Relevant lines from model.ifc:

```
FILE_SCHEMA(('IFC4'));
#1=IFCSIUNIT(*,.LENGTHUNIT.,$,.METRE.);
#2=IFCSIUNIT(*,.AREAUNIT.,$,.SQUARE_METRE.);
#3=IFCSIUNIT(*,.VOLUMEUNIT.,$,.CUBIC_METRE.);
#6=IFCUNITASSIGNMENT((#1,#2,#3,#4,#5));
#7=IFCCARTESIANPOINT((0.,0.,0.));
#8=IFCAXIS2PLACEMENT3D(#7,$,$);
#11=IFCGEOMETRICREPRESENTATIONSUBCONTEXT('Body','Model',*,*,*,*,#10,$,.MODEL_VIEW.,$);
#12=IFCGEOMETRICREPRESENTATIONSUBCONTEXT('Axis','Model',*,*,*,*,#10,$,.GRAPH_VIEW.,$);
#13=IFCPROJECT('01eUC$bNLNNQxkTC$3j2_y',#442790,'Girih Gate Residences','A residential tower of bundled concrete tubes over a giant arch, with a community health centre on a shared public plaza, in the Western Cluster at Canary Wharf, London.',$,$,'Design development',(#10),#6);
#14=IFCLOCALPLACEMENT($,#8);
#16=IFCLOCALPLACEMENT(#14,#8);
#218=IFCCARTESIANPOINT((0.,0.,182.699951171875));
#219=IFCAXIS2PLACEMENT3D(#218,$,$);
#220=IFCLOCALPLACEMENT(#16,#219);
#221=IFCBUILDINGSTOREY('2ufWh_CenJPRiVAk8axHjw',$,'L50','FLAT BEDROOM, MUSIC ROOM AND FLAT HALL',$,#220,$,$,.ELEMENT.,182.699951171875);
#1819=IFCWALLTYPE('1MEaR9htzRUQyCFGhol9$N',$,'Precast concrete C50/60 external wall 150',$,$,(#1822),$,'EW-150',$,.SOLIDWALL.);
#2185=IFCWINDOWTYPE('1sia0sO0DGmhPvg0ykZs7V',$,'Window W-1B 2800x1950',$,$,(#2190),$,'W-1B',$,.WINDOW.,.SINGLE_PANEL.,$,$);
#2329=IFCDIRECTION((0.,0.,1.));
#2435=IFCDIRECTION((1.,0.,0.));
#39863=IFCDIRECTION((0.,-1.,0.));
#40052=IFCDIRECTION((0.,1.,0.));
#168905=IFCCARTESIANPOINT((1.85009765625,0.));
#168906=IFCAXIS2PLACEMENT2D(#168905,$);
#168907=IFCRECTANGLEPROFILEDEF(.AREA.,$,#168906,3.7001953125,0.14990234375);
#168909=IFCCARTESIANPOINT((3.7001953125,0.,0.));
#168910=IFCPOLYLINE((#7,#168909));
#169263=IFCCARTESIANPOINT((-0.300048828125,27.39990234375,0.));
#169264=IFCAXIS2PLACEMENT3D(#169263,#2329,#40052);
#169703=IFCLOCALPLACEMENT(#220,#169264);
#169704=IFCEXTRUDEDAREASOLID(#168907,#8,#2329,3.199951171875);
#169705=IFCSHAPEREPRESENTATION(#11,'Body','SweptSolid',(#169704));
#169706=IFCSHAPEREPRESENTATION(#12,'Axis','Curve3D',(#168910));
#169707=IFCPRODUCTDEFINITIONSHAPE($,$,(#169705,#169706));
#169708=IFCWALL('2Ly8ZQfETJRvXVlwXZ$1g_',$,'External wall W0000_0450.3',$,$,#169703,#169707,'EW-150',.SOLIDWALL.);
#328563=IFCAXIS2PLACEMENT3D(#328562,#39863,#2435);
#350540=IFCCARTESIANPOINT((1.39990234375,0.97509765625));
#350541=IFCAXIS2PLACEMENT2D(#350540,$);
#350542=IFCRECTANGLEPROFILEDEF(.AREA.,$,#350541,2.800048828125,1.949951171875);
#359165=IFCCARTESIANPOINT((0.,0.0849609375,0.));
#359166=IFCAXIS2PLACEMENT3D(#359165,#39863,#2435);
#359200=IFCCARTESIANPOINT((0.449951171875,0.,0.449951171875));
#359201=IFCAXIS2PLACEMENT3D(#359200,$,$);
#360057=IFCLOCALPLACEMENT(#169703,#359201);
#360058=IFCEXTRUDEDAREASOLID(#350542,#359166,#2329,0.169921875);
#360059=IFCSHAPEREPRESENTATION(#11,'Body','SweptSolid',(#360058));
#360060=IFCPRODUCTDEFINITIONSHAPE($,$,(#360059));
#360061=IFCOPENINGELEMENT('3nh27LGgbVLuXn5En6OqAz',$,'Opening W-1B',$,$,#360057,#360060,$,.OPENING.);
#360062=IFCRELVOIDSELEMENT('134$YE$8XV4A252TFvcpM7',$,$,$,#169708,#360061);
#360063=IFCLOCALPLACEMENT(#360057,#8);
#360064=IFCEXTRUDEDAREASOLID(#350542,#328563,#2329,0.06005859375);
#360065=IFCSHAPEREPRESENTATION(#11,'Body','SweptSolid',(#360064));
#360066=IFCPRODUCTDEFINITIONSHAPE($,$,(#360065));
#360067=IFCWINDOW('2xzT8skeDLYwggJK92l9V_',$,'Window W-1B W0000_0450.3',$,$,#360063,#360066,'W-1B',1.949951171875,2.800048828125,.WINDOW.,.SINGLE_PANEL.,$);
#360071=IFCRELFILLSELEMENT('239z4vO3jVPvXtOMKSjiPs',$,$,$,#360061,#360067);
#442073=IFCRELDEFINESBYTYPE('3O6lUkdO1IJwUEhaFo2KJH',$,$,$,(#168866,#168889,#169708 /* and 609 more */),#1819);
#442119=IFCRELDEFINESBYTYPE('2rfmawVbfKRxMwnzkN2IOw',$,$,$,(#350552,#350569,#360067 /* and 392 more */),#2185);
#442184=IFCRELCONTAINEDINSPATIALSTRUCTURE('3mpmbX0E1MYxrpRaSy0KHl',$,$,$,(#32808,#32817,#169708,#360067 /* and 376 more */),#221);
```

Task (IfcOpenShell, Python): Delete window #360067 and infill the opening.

```python
import ifcopenshell
import ifcopenshell.api.feature
import ifcopenshell.api.root
import ifcopenshell.geom
import ifcopenshell.util.shape

model = ifcopenshell.open("model.ifc")
settings = ifcopenshell.geom.settings()


def volume(element):
    """Net volume in cubic metres, openings subtracted."""
    shape = ifcopenshell.geom.create_shape(settings, element)
    return ifcopenshell.util.shape.get_volume(shape.geometry)


window = model.by_guid("2xzT8skeDLYwggJK92l9V_")
opening = window.FillsVoids[0].RelatingOpeningElement
wall = opening.VoidsElements[0].RelatingBuildingElement
before = volume(wall)

ifcopenshell.api.root.remove_product(model, product=window)
ifcopenshell.api.feature.remove_feature(model, feature=opening)

after = volume(wall)

print(f"wall volume {before:.3f} -> {after:.3f} m3")

model.write("model_v2.ifc")
```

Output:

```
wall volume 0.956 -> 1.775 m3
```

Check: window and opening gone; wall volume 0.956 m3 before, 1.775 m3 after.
